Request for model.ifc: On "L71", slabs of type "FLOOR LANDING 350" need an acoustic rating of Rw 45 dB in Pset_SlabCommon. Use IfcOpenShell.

First a look at what the model holds.

```python
import ifcopenshell
import ifcopenshell.util.element

model = ifcopenshell.open("model.ifc")
print(model.schema)
storey = next(s for s in model.by_type("IfcBuildingStorey") if s.Name == "L71")
slabs = [e for e in ifcopenshell.util.element.get_decomposition(storey) if e.is_a("IfcSlab")]
seen = {}
for e in slabs:
    element_type = ifcopenshell.util.element.get_type(e)
    key = (element_type.Name if element_type != e and element_type else None, ifcopenshell.util.element.get_pset(e, "Pset_SlabCommon", "AcousticRating"))
    seen[key] = seen.get(key, 0) + 1
for (name, value), count in sorted(seen.items(), key=str):
    print(count, "x", name, "|", value)
```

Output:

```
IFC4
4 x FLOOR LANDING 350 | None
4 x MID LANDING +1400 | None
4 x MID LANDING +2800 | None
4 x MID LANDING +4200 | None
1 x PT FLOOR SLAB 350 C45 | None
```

```python
import ifcopenshell
import ifcopenshell.api.pset
import ifcopenshell.util.element

model = ifcopenshell.open("model.ifc")

storey = next(s for s in model.by_type("IfcBuildingStorey") if s.Name == "L71")
slabs = [e for e in ifcopenshell.util.element.get_decomposition(storey) if e.is_a("IfcSlab")]

count = 0
for e in slabs:
    element_type = ifcopenshell.util.element.get_type(e)
    if element_type in (None, e) or element_type.Name != "FLOOR LANDING 350":
        continue
    found = ifcopenshell.util.element.get_pset(e, "Pset_SlabCommon", should_inherit=False)
    if found:
        pset = model.by_id(found["id"])
        if len(ifcopenshell.util.element.get_elements_by_pset(pset)) > 1:
            pset = ifcopenshell.api.pset.unshare_pset(model, products=[e], pset=pset)[0]
    else:
        pset = ifcopenshell.api.pset.add_pset(model, product=e, name="Pset_SlabCommon")
    ifcopenshell.api.pset.edit_pset(model, pset=pset, properties={"AcousticRating": "Rw 45 dB"})
    count += 1

print(count, "slabs updated")

model.write("model_rev.ifc")
```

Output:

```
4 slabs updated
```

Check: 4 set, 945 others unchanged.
